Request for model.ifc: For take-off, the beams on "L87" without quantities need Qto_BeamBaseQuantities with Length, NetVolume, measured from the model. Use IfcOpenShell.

First a look at what the model holds.

```python
import ifcopenshell
import ifcopenshell.util.element
import ifcopenshell.util.unit

model = ifcopenshell.open("model.ifc")
print(model.schema)
for unit_type in ("LENGTHUNIT", "AREAUNIT", "VOLUMEUNIT"):
    print(unit_type, ifcopenshell.util.unit.calculate_unit_scale(model, unit_type))
storey = next(s for s in model.by_type("IfcBuildingStorey") if s.Name == "L87")
beams = [e for e in ifcopenshell.util.element.get_decomposition(storey) if e.is_a("IfcBeam")]
for e in sorted(beams, key=lambda e: e.id()):
    print(e.id(), e.is_a(), e.Name, list(ifcopenshell.util.element.get_psets(e, qtos_only=True)), sep=" | ")
```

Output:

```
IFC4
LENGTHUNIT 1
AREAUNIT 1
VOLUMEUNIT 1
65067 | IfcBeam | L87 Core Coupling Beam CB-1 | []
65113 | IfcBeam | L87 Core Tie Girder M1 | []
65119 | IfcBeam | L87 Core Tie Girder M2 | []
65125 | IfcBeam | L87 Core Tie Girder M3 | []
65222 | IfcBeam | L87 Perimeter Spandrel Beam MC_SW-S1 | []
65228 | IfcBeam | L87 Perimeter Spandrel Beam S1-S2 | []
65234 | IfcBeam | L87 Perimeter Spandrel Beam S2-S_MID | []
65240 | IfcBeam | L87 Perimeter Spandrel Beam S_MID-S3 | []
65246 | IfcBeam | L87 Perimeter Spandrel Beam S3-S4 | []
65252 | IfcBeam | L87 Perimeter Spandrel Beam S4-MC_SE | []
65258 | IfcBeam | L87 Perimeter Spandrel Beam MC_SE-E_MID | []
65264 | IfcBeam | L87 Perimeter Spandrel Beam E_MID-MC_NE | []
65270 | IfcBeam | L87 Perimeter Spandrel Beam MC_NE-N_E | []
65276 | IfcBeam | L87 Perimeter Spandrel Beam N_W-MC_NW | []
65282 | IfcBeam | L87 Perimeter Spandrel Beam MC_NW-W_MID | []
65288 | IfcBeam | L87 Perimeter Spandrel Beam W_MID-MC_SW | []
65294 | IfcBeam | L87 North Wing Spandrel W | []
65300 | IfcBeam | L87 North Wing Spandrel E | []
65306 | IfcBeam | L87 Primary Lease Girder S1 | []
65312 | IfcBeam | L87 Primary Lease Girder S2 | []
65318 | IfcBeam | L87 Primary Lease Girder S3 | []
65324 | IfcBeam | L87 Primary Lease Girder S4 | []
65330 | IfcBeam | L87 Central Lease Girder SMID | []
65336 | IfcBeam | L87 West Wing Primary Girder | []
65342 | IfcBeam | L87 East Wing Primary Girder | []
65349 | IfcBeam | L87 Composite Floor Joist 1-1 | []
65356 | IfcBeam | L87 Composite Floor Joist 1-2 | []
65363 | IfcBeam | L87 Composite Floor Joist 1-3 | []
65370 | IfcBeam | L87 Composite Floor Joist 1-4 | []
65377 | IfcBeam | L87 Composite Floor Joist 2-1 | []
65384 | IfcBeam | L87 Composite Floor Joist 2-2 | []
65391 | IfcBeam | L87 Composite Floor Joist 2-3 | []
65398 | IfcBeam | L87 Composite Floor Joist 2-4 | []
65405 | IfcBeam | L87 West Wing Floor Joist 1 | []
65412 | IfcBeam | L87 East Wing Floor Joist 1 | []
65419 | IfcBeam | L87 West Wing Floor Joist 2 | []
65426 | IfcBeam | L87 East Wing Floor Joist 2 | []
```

```python
import ifcopenshell
import ifcopenshell.api.pset
import ifcopenshell.geom
import ifcopenshell.util.element
import ifcopenshell.util.shape
import ifcopenshell.util.unit

model = ifcopenshell.open("model.ifc")
unit_scale = ifcopenshell.util.unit.calculate_unit_scale(model)
volume_scale = ifcopenshell.util.unit.calculate_unit_scale(model, "VOLUMEUNIT")
settings = ifcopenshell.geom.settings()

storey = next(s for s in model.by_type("IfcBuildingStorey") if s.Name == "L87")
beams = [e for e in ifcopenshell.util.element.get_decomposition(storey) if e.is_a("IfcBeam")]

for e in sorted(beams, key=lambda e: e.id()):
    if ifcopenshell.util.element.get_psets(e, qtos_only=True, should_inherit=False):
        continue
    # Geometry comes back in metres, in the element's own axes.
    shape = ifcopenshell.geom.create_shape(settings, e)
    values = {
        "Length": ifcopenshell.util.shape.get_max_xyz(shape.geometry) / unit_scale,
        "NetVolume": ifcopenshell.util.shape.get_volume(shape.geometry) / volume_scale,
    }
    qto = ifcopenshell.api.pset.add_qto(model, product=e, name="Qto_BeamBaseQuantities")
    ifcopenshell.api.pset.edit_qto(model, qto=qto, properties=values)
    print(e.id(), {k: round(v, 3) for k, v in values.items()})

model.write("model_updated.ifc")
```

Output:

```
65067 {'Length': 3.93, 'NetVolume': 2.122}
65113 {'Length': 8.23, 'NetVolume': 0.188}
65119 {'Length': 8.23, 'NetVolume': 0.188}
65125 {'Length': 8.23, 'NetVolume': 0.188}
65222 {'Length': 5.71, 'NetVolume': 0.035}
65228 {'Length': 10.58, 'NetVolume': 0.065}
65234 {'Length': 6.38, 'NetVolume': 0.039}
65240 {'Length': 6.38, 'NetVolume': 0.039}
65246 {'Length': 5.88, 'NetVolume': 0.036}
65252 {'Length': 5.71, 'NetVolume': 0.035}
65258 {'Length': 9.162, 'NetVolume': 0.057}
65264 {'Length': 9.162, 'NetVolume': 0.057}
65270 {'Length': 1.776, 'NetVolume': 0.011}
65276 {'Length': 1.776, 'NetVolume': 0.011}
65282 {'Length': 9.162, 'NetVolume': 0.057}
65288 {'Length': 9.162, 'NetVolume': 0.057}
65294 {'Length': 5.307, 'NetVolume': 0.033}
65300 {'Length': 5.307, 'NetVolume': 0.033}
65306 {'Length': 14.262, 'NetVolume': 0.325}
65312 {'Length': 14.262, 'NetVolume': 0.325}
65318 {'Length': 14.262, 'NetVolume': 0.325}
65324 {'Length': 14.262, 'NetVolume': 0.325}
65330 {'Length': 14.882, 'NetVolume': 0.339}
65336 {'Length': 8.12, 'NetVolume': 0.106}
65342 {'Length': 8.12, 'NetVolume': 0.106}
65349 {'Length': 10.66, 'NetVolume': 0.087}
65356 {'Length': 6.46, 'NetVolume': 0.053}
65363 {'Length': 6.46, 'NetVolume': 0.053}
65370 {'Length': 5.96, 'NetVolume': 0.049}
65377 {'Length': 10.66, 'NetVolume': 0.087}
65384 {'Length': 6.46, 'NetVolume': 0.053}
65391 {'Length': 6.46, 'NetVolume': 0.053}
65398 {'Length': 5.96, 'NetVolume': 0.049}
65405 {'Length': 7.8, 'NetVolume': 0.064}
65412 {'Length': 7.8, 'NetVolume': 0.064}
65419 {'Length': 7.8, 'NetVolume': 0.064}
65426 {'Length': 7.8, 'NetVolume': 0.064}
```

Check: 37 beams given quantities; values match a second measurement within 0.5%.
